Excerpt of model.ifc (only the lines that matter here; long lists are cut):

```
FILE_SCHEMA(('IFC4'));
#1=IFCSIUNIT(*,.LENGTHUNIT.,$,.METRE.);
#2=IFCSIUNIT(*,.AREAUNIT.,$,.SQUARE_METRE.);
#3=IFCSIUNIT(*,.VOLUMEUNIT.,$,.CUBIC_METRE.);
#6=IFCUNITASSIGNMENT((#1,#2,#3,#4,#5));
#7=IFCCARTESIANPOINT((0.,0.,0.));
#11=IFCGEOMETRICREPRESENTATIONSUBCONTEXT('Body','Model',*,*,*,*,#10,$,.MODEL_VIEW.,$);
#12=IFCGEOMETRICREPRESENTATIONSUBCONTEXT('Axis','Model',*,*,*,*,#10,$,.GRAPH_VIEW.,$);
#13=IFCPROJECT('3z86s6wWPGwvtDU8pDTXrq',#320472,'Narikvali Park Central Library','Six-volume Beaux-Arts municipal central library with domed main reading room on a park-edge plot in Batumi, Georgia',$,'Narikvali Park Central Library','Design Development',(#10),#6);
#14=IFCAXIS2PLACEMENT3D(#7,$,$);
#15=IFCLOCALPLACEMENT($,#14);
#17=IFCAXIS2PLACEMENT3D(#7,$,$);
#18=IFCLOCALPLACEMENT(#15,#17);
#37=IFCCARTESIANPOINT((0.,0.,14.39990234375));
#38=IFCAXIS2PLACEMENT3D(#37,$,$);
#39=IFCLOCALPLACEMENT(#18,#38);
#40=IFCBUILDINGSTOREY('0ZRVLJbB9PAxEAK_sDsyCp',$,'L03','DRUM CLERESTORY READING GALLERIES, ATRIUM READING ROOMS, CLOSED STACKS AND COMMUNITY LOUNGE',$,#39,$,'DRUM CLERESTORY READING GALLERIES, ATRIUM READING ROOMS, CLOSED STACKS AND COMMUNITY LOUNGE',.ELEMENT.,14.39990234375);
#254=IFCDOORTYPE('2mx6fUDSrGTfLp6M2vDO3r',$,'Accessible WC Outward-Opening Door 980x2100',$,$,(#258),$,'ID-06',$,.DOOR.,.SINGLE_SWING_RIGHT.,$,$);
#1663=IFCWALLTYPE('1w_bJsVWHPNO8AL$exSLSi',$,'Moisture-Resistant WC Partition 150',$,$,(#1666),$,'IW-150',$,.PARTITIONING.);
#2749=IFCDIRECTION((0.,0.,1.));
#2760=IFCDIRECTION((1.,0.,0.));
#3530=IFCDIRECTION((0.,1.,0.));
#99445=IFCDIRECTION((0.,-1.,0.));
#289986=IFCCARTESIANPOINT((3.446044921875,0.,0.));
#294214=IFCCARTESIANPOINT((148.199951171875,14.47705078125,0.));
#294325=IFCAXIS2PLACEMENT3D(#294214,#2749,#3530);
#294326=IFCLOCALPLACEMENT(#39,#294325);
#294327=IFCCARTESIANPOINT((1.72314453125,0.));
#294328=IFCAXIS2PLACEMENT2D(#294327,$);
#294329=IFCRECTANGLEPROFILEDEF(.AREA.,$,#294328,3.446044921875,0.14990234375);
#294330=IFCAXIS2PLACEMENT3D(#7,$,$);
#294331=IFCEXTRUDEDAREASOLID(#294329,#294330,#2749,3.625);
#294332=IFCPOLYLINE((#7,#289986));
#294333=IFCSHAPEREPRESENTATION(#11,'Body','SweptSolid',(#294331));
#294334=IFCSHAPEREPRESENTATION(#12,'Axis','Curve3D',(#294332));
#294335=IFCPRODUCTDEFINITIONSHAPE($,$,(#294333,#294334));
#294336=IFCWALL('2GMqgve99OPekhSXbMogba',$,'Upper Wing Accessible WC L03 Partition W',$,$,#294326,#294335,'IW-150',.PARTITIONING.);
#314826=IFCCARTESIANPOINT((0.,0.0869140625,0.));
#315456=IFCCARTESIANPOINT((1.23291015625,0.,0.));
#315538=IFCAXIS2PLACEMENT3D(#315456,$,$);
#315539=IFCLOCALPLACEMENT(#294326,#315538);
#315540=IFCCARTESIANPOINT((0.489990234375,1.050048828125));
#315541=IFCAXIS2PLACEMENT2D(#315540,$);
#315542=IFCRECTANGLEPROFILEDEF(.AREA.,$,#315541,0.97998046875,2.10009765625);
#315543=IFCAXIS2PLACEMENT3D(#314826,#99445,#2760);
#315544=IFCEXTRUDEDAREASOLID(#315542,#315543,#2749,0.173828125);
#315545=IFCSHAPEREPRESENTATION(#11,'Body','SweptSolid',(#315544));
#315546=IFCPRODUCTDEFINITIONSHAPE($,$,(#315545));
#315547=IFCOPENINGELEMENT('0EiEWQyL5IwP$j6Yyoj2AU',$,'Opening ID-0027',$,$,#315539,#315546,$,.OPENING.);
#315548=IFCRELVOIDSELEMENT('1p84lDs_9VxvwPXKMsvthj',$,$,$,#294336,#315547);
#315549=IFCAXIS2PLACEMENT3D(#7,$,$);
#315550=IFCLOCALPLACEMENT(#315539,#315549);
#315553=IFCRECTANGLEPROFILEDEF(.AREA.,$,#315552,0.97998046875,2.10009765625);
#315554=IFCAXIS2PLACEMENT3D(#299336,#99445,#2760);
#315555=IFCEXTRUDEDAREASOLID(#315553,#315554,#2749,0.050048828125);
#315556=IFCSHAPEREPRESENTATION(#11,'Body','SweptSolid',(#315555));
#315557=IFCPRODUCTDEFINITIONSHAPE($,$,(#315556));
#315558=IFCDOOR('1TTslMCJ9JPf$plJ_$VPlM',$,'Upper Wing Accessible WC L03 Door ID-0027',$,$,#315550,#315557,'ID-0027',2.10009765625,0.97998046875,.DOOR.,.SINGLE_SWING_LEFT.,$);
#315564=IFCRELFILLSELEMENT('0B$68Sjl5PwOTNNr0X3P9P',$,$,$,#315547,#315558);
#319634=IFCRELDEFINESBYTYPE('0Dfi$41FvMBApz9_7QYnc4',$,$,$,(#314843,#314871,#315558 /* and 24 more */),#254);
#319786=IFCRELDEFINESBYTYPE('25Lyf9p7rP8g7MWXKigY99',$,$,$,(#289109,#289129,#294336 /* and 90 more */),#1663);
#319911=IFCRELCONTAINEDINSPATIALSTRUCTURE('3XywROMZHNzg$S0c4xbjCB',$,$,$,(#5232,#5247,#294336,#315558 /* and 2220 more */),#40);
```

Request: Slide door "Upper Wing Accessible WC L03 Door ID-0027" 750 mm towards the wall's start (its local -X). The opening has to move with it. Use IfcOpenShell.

```python
import ifcopenshell
import ifcopenshell.api.geometry
import ifcopenshell.util.placement
import ifcopenshell.util.unit

model = ifcopenshell.open("model.ifc")
unit_scale = ifcopenshell.util.unit.calculate_unit_scale(model)

door = model.by_guid("1TTslMCJ9JPf$plJ_$VPlM")
opening = door.FillsVoids[0].RelatingOpeningElement
wall = opening.VoidsElements[0].RelatingBuildingElement

wall_matrix = ifcopenshell.util.placement.get_local_placement(wall.ObjectPlacement)
shift = wall_matrix[:3, 0] * -0.75 / unit_scale
before = ifcopenshell.util.placement.get_local_placement(door.ObjectPlacement)[:3, 3].copy()

# The door is placed relative to its opening, so it follows when the opening moves.
matrix = ifcopenshell.util.placement.get_local_placement(opening.ObjectPlacement)
matrix[:3, 3] += shift
ifcopenshell.api.geometry.edit_object_placement(
    model, product=opening, matrix=matrix, is_si=False, should_transform_children=True
)

after = ifcopenshell.util.placement.get_local_placement(door.ObjectPlacement)[:3, 3]
print("door moved by", (after - before).round(3) + 0.0)

model.write("model-out.ifc")
```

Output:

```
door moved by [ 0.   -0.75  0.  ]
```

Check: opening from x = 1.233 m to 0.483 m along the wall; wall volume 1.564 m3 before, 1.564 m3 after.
